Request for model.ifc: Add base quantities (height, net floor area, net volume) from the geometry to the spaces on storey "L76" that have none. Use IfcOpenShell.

First a look at what the model holds.

```python
import ifcopenshell
import ifcopenshell.util.element
import ifcopenshell.util.unit

model = ifcopenshell.open("model.ifc")
print(model.schema)
for unit_type in ("LENGTHUNIT", "AREAUNIT", "VOLUMEUNIT"):
    print(unit_type, ifcopenshell.util.unit.calculate_unit_scale(model, unit_type))
storey = next(s for s in model.by_type("IfcBuildingStorey") if s.Name == "L76")
spaces = [e for e in ifcopenshell.util.element.get_decomposition(storey) if e.is_a("IfcSpace")]
for e in sorted(spaces, key=lambda e: e.id()):
    print(e.id(), e.is_a(), e.Name, list(ifcopenshell.util.element.get_psets(e, qtos_only=True)), sep=" | ")
```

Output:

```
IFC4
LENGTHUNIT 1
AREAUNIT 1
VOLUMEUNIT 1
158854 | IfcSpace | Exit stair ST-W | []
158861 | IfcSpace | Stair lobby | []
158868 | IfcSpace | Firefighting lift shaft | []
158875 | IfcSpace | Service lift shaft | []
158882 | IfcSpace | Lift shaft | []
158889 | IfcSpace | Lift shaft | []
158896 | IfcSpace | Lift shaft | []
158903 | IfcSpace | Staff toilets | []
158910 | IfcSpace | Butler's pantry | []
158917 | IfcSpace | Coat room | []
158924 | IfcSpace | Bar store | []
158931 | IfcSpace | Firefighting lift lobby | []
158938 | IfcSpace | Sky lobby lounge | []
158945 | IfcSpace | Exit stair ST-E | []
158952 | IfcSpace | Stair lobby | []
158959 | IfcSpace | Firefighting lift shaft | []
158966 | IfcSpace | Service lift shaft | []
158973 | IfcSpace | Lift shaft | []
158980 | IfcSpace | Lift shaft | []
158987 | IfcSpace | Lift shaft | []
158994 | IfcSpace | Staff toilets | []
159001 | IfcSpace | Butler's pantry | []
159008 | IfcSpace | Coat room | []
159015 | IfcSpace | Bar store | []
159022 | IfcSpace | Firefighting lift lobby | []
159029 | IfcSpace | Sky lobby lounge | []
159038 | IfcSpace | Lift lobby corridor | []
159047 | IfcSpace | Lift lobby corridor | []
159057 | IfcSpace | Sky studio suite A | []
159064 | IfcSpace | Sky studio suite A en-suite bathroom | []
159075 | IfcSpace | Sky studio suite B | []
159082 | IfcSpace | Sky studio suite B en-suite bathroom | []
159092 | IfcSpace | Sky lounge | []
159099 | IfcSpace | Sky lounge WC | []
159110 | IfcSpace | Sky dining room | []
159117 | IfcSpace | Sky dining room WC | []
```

```python
import ifcopenshell
import ifcopenshell.api.pset
import ifcopenshell.geom
import ifcopenshell.util.element
import ifcopenshell.util.shape
import ifcopenshell.util.unit

model = ifcopenshell.open("model.ifc")
unit_scale = ifcopenshell.util.unit.calculate_unit_scale(model)
area_scale = ifcopenshell.util.unit.calculate_unit_scale(model, "AREAUNIT")
volume_scale = ifcopenshell.util.unit.calculate_unit_scale(model, "VOLUMEUNIT")
settings = ifcopenshell.geom.settings()

storey = next(s for s in model.by_type("IfcBuildingStorey") if s.Name == "L76")
spaces = [e for e in ifcopenshell.util.element.get_decomposition(storey) if e.is_a("IfcSpace")]

for e in sorted(spaces, key=lambda e: e.id()):
    if ifcopenshell.util.element.get_psets(e, qtos_only=True, should_inherit=False):
        continue
    # Geometry comes back in metres, in the element's own axes.
    shape = ifcopenshell.geom.create_shape(settings, e)
    values = {
        "Height": ifcopenshell.util.shape.get_z(shape.geometry) / unit_scale,
        "NetFloorArea": ifcopenshell.util.shape.get_footprint_area(shape.geometry) / area_scale,
        "NetVolume": ifcopenshell.util.shape.get_volume(shape.geometry) / volume_scale,
    }
    qto = ifcopenshell.api.pset.add_qto(model, product=e, name="Qto_SpaceBaseQuantities")
    ifcopenshell.api.pset.edit_qto(model, qto=qto, properties=values)
    print(e.id(), {k: round(v, 3) for k, v in values.items()})

model.write("model-out.ifc")
```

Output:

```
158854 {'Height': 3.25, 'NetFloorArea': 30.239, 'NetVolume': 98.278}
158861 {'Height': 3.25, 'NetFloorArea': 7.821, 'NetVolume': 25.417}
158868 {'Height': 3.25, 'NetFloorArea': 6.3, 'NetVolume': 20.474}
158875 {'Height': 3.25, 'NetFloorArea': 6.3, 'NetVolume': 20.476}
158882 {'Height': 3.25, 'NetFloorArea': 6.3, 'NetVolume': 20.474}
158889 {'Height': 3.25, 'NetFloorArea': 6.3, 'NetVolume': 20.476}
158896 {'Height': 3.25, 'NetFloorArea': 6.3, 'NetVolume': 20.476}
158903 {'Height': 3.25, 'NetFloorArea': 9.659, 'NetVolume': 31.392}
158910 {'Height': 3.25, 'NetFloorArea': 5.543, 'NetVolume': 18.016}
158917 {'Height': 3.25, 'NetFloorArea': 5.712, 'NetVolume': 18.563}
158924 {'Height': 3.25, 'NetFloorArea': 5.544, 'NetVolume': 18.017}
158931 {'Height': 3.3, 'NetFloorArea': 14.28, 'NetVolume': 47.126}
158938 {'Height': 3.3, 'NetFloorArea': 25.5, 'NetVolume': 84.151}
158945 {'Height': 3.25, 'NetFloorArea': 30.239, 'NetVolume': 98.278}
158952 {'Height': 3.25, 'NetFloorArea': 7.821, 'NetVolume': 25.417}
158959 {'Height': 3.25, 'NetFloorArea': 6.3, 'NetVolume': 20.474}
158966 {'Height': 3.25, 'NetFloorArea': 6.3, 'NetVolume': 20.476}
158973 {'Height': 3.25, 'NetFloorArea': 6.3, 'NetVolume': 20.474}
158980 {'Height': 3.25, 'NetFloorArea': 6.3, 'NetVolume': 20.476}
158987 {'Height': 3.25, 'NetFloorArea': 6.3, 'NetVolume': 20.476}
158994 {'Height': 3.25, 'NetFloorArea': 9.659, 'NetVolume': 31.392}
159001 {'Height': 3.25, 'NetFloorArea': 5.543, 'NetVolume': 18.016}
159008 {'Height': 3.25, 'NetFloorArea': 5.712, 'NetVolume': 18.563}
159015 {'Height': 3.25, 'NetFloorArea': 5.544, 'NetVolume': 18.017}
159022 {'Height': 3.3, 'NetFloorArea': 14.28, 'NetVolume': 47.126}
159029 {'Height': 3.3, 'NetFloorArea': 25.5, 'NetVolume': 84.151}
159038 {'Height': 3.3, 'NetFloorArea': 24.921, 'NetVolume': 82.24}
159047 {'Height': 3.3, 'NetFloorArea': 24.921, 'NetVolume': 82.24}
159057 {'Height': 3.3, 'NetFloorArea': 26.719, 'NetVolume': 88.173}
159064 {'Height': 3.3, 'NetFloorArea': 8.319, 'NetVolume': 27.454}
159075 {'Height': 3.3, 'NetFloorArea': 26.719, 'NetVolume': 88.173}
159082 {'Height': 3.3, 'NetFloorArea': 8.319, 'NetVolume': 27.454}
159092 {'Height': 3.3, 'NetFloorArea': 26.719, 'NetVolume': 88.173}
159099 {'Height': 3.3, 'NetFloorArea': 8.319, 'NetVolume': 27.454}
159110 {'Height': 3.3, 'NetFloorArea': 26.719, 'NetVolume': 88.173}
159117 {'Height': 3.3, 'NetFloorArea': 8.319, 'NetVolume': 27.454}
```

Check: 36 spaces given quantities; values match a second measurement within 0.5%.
